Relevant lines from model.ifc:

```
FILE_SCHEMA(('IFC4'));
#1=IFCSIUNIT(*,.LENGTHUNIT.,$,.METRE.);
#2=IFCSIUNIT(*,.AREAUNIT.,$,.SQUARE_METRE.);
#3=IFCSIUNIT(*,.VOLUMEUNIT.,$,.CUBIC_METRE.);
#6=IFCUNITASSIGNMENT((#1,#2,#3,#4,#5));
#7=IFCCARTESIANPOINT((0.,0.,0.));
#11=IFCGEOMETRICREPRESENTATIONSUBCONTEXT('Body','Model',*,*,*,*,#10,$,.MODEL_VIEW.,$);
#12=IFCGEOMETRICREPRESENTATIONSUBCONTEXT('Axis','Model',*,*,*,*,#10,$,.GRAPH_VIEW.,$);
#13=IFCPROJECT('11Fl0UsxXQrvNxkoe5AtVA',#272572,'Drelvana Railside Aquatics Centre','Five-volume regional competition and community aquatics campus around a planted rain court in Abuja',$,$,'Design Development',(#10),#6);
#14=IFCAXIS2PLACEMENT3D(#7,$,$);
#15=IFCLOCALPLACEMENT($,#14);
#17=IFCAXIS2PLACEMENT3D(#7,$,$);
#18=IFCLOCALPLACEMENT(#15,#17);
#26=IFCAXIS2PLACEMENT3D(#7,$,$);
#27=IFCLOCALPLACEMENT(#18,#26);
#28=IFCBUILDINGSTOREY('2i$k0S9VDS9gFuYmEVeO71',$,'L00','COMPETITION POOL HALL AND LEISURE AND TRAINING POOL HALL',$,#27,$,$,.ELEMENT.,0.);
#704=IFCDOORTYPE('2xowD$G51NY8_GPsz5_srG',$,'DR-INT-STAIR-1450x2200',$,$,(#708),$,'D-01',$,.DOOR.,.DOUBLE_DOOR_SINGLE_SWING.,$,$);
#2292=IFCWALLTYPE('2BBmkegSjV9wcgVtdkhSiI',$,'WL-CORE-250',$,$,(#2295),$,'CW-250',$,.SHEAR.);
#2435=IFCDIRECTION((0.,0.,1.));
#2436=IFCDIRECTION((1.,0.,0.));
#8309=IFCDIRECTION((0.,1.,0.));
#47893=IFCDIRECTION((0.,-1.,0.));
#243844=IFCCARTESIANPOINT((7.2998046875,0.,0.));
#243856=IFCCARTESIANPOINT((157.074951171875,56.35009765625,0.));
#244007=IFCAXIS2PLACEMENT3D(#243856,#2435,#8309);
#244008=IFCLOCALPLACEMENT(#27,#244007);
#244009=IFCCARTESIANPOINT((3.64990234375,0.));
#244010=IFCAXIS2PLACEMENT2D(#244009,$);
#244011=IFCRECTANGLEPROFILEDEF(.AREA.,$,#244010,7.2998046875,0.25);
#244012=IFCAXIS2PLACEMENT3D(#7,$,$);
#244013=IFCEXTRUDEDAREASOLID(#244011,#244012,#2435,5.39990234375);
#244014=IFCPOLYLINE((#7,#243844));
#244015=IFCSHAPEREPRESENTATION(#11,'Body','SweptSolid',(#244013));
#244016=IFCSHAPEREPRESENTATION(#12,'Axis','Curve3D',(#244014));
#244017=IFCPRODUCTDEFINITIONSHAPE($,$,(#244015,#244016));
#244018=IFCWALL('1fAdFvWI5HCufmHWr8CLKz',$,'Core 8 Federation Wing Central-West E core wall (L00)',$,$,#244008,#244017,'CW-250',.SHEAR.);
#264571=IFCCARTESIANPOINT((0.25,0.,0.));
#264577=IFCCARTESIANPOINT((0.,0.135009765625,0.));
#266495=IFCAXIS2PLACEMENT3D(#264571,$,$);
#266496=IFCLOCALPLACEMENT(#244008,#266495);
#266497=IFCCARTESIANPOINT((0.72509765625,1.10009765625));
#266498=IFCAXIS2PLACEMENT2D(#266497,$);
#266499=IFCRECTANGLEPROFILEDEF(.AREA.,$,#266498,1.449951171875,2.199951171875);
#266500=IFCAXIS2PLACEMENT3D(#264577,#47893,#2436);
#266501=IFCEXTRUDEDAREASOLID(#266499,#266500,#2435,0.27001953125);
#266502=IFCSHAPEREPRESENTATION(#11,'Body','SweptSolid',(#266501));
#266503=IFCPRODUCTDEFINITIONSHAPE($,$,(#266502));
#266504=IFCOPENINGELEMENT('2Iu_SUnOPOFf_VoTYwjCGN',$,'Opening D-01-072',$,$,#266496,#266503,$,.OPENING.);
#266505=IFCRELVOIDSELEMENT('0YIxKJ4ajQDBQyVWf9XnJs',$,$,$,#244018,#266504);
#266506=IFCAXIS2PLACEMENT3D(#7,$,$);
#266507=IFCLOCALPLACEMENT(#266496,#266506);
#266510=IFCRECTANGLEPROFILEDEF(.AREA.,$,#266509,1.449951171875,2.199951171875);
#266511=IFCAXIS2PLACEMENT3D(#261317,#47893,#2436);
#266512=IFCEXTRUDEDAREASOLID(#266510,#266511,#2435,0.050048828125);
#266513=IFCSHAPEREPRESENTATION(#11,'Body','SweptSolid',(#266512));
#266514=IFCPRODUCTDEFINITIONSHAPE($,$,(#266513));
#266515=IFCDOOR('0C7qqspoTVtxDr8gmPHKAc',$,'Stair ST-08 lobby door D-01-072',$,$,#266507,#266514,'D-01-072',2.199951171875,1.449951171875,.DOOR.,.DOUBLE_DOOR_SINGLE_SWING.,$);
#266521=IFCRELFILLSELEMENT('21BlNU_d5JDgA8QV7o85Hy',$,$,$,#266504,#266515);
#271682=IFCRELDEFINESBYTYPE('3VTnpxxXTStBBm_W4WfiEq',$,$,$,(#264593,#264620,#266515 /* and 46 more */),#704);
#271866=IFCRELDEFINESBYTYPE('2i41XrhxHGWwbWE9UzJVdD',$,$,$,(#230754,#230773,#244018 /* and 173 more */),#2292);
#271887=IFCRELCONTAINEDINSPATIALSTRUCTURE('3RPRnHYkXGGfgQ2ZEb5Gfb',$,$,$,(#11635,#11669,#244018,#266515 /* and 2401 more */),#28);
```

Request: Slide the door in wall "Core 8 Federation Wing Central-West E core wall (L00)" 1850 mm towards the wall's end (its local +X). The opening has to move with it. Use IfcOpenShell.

```python
import ifcopenshell
import ifcopenshell.api.geometry
import ifcopenshell.util.placement
import ifcopenshell.util.unit

model = ifcopenshell.open("model.ifc")
unit_scale = ifcopenshell.util.unit.calculate_unit_scale(model)

door = model.by_id(266515)
opening = door.FillsVoids[0].RelatingOpeningElement
wall = opening.VoidsElements[0].RelatingBuildingElement

wall_matrix = ifcopenshell.util.placement.get_local_placement(wall.ObjectPlacement)
shift = wall_matrix[:3, 0] * 1.85 / unit_scale
before = ifcopenshell.util.placement.get_local_placement(door.ObjectPlacement)[:3, 3].copy()

# The door is placed relative to its opening, so it follows when the opening moves.
matrix = ifcopenshell.util.placement.get_local_placement(opening.ObjectPlacement)
matrix[:3, 3] += shift
ifcopenshell.api.geometry.edit_object_placement(
    model, product=opening, matrix=matrix, is_si=False, should_transform_children=True
)

after = ifcopenshell.util.placement.get_local_placement(door.ObjectPlacement)[:3, 3]
print("door moved by", (after - before).round(3) + 0.0)

model.write("model-out.ifc")
```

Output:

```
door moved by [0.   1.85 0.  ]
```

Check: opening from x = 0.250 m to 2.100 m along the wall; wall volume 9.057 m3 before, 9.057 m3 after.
